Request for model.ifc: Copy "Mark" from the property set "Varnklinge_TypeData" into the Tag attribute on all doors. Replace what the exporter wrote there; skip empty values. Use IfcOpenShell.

First a look at what the model holds.

```python
import ifcopenshell
import ifcopenshell.util.element

model = ifcopenshell.open("model.ifc")
print(model.schema)
doors = model.by_type("IfcDoor")
print(len(doors), "doors")
for e in doors[:8]:
    source = ifcopenshell.util.element.get_pset(e, "Varnklinge_TypeData", "Mark")
    target = e.Tag
    print(e.id(), repr(source), repr(target), sep=" | ")
```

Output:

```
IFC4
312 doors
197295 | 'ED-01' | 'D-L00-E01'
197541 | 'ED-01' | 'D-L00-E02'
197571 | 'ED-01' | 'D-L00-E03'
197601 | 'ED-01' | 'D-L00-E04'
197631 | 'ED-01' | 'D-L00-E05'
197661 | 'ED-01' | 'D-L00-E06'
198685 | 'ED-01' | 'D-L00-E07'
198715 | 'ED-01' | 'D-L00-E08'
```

```python
import ifcopenshell
import ifcopenshell.util.element

model = ifcopenshell.open("model.ifc")

count = 0
for e in model.by_type("IfcDoor"):
    value = ifcopenshell.util.element.get_pset(e, "Varnklinge_TypeData", "Mark")
    current = e.Tag
    if not value or not value.strip() or current == value:
        continue
    e.Tag = value
    count += 1

print(count, "doors updated")

model.write("model_updated.ifc")
```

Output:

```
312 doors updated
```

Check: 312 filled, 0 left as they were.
